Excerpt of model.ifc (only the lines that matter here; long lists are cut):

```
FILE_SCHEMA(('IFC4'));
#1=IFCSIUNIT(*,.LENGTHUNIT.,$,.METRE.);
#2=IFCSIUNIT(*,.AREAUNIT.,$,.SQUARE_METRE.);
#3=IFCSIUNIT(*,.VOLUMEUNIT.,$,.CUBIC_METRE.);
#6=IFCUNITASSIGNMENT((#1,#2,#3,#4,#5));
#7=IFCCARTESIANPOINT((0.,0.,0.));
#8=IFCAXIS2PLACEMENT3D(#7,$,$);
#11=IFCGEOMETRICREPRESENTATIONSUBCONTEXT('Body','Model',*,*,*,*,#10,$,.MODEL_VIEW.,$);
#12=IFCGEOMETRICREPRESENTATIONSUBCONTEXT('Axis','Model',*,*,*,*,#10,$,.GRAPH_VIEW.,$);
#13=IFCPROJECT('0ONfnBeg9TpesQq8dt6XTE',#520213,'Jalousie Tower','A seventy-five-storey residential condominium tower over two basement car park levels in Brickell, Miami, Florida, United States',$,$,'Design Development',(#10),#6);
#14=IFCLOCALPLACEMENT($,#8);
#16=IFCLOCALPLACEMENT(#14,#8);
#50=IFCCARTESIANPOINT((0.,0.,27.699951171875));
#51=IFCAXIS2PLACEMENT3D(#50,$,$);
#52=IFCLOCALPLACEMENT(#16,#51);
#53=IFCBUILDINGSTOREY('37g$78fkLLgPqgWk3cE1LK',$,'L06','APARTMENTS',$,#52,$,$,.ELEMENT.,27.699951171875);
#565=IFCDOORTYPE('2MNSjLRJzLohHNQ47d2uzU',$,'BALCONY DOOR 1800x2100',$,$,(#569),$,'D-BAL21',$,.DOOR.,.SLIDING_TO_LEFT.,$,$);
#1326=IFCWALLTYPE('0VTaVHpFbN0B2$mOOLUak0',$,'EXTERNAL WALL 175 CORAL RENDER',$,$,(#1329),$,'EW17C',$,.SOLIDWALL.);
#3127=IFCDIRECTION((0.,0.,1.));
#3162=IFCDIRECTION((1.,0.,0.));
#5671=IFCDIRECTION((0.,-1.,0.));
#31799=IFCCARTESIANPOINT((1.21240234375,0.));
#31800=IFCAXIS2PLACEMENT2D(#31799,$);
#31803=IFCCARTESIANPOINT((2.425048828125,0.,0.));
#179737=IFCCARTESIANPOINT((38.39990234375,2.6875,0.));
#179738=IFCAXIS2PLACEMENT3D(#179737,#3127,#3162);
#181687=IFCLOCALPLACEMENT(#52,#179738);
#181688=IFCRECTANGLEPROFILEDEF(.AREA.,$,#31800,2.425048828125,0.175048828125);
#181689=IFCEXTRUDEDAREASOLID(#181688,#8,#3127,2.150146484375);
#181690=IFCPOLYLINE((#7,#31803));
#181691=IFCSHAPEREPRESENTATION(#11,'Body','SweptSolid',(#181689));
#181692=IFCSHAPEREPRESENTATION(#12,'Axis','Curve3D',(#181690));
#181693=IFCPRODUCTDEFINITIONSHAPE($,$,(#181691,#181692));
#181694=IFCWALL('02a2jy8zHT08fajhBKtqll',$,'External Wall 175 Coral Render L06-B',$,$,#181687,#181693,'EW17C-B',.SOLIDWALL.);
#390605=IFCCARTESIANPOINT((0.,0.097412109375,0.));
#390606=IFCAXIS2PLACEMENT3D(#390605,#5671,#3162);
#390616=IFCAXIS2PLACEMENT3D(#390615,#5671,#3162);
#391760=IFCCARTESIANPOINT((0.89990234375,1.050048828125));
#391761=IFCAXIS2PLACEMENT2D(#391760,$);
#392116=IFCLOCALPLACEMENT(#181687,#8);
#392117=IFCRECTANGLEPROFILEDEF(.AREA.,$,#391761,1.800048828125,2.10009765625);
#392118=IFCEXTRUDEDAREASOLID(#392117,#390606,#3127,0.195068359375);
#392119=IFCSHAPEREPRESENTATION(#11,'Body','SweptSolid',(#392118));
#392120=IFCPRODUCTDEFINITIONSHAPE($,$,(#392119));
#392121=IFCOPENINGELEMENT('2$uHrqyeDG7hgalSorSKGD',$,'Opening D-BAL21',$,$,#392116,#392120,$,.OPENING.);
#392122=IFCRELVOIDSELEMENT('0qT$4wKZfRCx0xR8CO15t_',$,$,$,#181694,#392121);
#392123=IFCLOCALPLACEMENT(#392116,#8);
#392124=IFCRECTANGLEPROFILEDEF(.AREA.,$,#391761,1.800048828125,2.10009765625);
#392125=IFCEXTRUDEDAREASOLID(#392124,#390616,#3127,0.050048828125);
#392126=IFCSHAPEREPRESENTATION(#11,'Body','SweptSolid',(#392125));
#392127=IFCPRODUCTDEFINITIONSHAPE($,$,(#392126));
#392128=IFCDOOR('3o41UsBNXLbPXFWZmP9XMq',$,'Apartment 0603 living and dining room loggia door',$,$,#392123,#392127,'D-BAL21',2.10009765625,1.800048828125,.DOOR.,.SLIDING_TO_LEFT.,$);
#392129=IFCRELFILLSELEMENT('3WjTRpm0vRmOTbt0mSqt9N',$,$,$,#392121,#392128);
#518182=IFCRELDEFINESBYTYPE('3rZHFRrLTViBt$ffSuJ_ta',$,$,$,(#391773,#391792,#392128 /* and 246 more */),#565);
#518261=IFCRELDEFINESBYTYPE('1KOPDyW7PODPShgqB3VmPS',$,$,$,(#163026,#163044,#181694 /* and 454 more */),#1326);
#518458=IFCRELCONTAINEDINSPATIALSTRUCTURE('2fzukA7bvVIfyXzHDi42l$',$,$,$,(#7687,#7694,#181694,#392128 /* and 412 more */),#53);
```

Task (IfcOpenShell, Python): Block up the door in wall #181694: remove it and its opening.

```python
import ifcopenshell
import ifcopenshell.api.feature
import ifcopenshell.api.root
import ifcopenshell.geom
import ifcopenshell.util.shape

model = ifcopenshell.open("model.ifc")
settings = ifcopenshell.geom.settings()


def volume(element):
    """Net volume in cubic metres, openings subtracted."""
    shape = ifcopenshell.geom.create_shape(settings, element)
    return ifcopenshell.util.shape.get_volume(shape.geometry)


door = model.by_guid("3o41UsBNXLbPXFWZmP9XMq")
opening = door.FillsVoids[0].RelatingOpeningElement
wall = opening.VoidsElements[0].RelatingBuildingElement
before = volume(wall)

ifcopenshell.api.root.remove_product(model, product=door)
ifcopenshell.api.feature.remove_feature(model, feature=opening)

after = volume(wall)

print(f"wall volume {before:.3f} -> {after:.3f} m3")

model.write("model_edited.ifc")
```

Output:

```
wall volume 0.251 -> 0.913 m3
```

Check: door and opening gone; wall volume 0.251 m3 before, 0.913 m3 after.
